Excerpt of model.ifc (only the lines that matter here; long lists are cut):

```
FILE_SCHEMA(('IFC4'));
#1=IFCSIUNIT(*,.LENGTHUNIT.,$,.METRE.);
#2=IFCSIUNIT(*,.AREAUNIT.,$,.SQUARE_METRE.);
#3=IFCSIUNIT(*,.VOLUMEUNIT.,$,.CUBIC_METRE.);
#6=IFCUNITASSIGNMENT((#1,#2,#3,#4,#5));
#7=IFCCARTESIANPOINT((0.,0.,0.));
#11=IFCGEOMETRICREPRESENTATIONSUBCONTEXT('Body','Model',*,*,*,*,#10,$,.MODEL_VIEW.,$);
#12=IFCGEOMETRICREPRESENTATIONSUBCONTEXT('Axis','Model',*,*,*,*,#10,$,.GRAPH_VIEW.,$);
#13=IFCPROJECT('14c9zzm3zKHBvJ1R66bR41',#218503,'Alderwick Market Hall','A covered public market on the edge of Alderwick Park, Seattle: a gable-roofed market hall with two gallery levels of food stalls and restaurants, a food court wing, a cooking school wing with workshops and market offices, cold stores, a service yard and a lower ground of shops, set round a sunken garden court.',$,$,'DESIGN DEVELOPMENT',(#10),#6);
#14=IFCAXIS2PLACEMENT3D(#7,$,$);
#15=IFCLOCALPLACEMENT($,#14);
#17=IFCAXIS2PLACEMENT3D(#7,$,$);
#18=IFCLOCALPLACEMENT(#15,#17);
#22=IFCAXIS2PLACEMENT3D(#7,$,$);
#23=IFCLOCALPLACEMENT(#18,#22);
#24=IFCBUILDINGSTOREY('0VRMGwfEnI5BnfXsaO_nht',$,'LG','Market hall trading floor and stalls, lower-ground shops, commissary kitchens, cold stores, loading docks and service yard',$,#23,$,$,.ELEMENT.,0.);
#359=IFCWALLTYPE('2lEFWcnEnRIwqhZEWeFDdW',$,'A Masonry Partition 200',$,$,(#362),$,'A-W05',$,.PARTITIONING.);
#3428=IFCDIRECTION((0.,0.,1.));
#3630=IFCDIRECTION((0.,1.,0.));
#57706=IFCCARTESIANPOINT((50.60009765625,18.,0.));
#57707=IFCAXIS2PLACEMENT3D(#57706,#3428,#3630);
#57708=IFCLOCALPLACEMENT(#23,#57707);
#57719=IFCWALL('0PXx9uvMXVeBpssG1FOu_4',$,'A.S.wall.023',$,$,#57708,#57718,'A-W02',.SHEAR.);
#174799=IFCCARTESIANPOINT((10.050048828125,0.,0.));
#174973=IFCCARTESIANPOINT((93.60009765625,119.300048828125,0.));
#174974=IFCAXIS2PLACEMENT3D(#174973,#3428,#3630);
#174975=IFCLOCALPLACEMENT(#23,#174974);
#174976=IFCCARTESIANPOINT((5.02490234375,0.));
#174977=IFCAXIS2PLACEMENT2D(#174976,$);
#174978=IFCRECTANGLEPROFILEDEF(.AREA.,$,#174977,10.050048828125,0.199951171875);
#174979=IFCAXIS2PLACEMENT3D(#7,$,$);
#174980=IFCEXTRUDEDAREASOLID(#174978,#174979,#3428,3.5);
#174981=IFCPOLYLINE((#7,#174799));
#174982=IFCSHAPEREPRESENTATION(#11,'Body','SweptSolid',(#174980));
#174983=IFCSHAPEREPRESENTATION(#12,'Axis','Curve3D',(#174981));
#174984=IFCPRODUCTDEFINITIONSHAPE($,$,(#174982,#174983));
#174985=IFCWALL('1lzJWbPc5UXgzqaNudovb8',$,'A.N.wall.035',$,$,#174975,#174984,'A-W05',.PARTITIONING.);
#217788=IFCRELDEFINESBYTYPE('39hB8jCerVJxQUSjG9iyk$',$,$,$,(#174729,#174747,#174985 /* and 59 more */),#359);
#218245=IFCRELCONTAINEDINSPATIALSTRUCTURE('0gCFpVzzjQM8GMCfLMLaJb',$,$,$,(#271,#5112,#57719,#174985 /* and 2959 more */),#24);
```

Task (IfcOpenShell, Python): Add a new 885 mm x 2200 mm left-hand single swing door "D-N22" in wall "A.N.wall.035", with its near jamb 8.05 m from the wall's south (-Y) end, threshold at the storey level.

```python
import numpy as np
import ifcopenshell
import ifcopenshell.api.feature
import ifcopenshell.api.geometry
import ifcopenshell.api.root
import ifcopenshell.api.spatial
import ifcopenshell.geom
import ifcopenshell.util.element
import ifcopenshell.util.placement
import ifcopenshell.util.representation
import ifcopenshell.util.shape
import ifcopenshell.util.unit

model = ifcopenshell.open("model.ifc")
unit_scale = ifcopenshell.util.unit.calculate_unit_scale(model)
settings = ifcopenshell.geom.settings()


def volume(element):
    """Net volume in cubic metres, openings subtracted."""
    shape = ifcopenshell.geom.create_shape(settings, element)
    return ifcopenshell.util.shape.get_volume(shape.geometry)


wall = model.by_guid("1lzJWbPc5UXgzqaNudovb8")
storey = ifcopenshell.util.element.get_container(wall, ifc_class="IfcBuildingStorey")
context = ifcopenshell.util.representation.get_context(model, "Model", "Body", "MODEL_VIEW")
before = volume(wall)

width, height, from_end, sill = 0.885, 2.2, 8.05, 0.0  # metres

# The wall runs along its own X axis, and the end named is its -X end.
wall_shape = ifcopenshell.geom.create_shape(settings, wall)
x, y, z = ifcopenshell.util.shape.get_vertices(wall_shape.geometry).T
start = x.min() + from_end
face, thickness = float(y.min()), float(y.max() - y.min())
wall_matrix = ifcopenshell.util.placement.get_local_placement(wall.ObjectPlacement)
level = ifcopenshell.util.placement.get_local_placement(storey.ObjectPlacement)[2, 3]


def in_wall(x, y):
    """Placement at x, y metres in the wall's axes, at sill height."""
    matrix = wall_matrix.copy()
    matrix[:, 3] = wall_matrix @ np.array([x / unit_scale, y / unit_scale, 0.0, 1.0])
    matrix[2, 3] = level + sill / unit_scale
    return matrix


# Opening: a box that overshoots both wall faces by 50 mm.
opening = ifcopenshell.api.root.create_entity(model, ifc_class="IfcOpeningElement", predefined_type="OPENING")
box = ifcopenshell.api.geometry.add_wall_representation(
    model, context=context, length=width, height=height, thickness=thickness + 0.1
)
ifcopenshell.api.geometry.assign_representation(model, product=opening, representation=box)
ifcopenshell.api.geometry.edit_object_placement(model, product=opening, matrix=in_wall(start, face - 0.05), is_si=False)
ifcopenshell.api.feature.add_feature(model, feature=opening, element=wall)

door = ifcopenshell.api.root.create_entity(model, ifc_class="IfcDoor", name="D-N22", predefined_type="DOOR")
door.OverallWidth, door.OverallHeight = width / unit_scale, height / unit_scale
door.OperationType = "SINGLE_SWING_LEFT"
body = ifcopenshell.api.geometry.add_door_representation(
    model,
    context=context,
    overall_width=door.OverallWidth,
    overall_height=door.OverallHeight,
    operation_type="SINGLE_SWING_LEFT",
    lining_properties={"LiningDepth": thickness / unit_scale, "ThresholdDepth": thickness / unit_scale},
)
ifcopenshell.api.geometry.assign_representation(model, product=door, representation=body)
ifcopenshell.api.spatial.assign_container(model, products=[door], relating_structure=storey)
ifcopenshell.api.feature.add_filling(model, opening=opening, element=door)

# The lining spans the wall, so the door starts at the wall face.
ifcopenshell.api.geometry.edit_object_placement(model, product=door, matrix=in_wall(start, face), is_si=False)

after = volume(wall)

print(f"wall volume {before:.3f} -> {after:.3f} m3")

model.write("model_v2.ifc")
```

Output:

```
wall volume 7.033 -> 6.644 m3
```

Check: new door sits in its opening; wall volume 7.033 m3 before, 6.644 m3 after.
